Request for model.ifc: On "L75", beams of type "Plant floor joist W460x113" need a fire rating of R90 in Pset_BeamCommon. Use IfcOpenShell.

First a look at what the model holds.

```python
import ifcopenshell
import ifcopenshell.util.element

model = ifcopenshell.open("model.ifc")
print(model.schema)
storey = next(s for s in model.by_type("IfcBuildingStorey") if s.Name == "L75")
beams = [e for e in ifcopenshell.util.element.get_decomposition(storey) if e.is_a("IfcBeam")]
seen = {}
for e in beams:
    element_type = ifcopenshell.util.element.get_type(e)
    key = (element_type.Name if element_type != e and element_type else None, ifcopenshell.util.element.get_pset(e, "Pset_BeamCommon", "FireRating"))
    seen[key] = seen.get(key, 0) + 1
for (name, value), count in sorted(seen.items(), key=str):
    print(count, "x", name, "|", value)
```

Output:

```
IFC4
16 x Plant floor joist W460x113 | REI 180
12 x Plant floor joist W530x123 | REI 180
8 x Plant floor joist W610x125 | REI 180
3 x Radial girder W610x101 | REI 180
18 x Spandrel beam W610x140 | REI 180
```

```python
import ifcopenshell
import ifcopenshell.api.pset
import ifcopenshell.util.element

model = ifcopenshell.open("model.ifc")

storey = next(s for s in model.by_type("IfcBuildingStorey") if s.Name == "L75")
beams = [e for e in ifcopenshell.util.element.get_decomposition(storey) if e.is_a("IfcBeam")]

count = 0
for e in beams:
    element_type = ifcopenshell.util.element.get_type(e)
    if element_type in (None, e) or element_type.Name != "Plant floor joist W460x113":
        continue
    found = ifcopenshell.util.element.get_pset(e, "Pset_BeamCommon", should_inherit=False)
    if found:
        pset = model.by_id(found["id"])
        if len(ifcopenshell.util.element.get_elements_by_pset(pset)) > 1:
            pset = ifcopenshell.api.pset.unshare_pset(model, products=[e], pset=pset)[0]
    else:
        pset = ifcopenshell.api.pset.add_pset(model, product=e, name="Pset_BeamCommon")
    ifcopenshell.api.pset.edit_pset(model, pset=pset, properties={"FireRating": "R90"})
    count += 1

print(count, "beams updated")

model.write("model_updated.ifc")
```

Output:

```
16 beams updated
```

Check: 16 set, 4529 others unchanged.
